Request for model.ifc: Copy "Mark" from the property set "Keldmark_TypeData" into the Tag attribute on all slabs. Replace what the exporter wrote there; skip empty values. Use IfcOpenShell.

First a look at what the model holds.

```python
import ifcopenshell
import ifcopenshell.util.element

model = ifcopenshell.open("model.ifc")
print(model.schema)
slabs = model.by_type("IfcSlab")
print(len(slabs), "slabs")
for e in slabs[:8]:
    source = ifcopenshell.util.element.get_pset(e, "Keldmark_TypeData", "Mark")
    target = e.Tag
    print(e.id(), repr(source), repr(target), sep=" | ")
```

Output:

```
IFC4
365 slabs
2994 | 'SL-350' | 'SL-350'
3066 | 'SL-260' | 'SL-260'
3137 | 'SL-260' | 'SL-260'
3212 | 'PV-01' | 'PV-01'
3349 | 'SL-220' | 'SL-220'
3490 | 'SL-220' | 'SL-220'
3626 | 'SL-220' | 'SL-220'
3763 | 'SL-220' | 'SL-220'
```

```python
import ifcopenshell
import ifcopenshell.util.element

model = ifcopenshell.open("model.ifc")

count = 0
for e in model.by_type("IfcSlab"):
    value = ifcopenshell.util.element.get_pset(e, "Keldmark_TypeData", "Mark")
    current = e.Tag
    if not value or not value.strip() or current == value:
        continue
    e.Tag = value
    count += 1

print(count, "slabs updated")

model.write("model_rev.ifc")
```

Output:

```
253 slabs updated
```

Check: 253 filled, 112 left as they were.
